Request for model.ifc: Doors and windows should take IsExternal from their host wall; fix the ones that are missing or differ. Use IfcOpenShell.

First a look at what the model holds.

```python
import ifcopenshell
import ifcopenshell.util.element

model = ifcopenshell.open("model.ifc")
print(model.schema)
seen = {}
for e in model.by_type("IfcDoor") + model.by_type("IfcWindow"):
    if not e.FillsVoids:
        continue
    host = e.FillsVoids[0].RelatingOpeningElement.VoidsElements[0].RelatingBuildingElement
    own = ifcopenshell.util.element.get_pset(e, f"Pset_{e.is_a()[3:].removesuffix('StandardCase')}Common", "IsExternal")
    wall = ifcopenshell.util.element.get_pset(host, "Pset_WallCommon", "IsExternal")
    seen[e.is_a(), own, wall] = seen.get((e.is_a(), own, wall), 0) + 1
for (cls, own, wall), count in sorted(seen.items(), key=str):
    print(count, cls, "IsExternal:", own, "| host wall:", wall)
```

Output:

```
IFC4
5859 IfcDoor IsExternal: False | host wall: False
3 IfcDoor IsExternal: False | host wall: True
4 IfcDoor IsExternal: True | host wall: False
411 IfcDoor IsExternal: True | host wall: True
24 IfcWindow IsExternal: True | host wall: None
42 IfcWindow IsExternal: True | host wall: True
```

```python
import ifcopenshell
import ifcopenshell.api.pset
import ifcopenshell.util.element

model = ifcopenshell.open("model.ifc")

count = 0
for ifc_class, pset_name in (("IfcDoor", "Pset_DoorCommon"), ("IfcWindow", "Pset_WindowCommon")):
    for e in model.by_type(ifc_class):
        if not e.FillsVoids:
            continue
        host = e.FillsVoids[0].RelatingOpeningElement.VoidsElements[0].RelatingBuildingElement
        external = ifcopenshell.util.element.get_pset(host, "Pset_WallCommon", "IsExternal")
        if external is None or ifcopenshell.util.element.get_pset(e, pset_name, "IsExternal") == external:
            continue
        pset = ifcopenshell.api.pset.add_pset(model, product=e, name=pset_name)
        ifcopenshell.api.pset.edit_pset(model, pset=pset, properties={"IsExternal": external})
        count += 1

print(count, "updated")

model.write("model_updated.ifc")
```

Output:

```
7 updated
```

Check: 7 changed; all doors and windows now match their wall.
